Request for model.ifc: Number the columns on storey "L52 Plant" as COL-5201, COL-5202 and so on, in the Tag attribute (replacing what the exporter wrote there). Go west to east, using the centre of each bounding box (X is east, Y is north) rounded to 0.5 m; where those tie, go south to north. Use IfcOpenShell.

First a look at what the model holds.

```python
import ifcopenshell
import ifcopenshell.util.element
import ifcopenshell.util.placement

model = ifcopenshell.open("model.ifc")
print(model.schema)
storey = next(s for s in model.by_type("IfcBuildingStorey") if s.Name == "L52 Plant")
columns = [e for e in ifcopenshell.util.element.get_decomposition(storey) if e.is_a("IfcColumn")]
for e in sorted(columns, key=lambda e: e.id()):
    origin = ifcopenshell.util.placement.get_local_placement(e.ObjectPlacement)[:3, 3]
    print(e.id(), e.Tag, e.Name, origin.round(2) + 0.0, sep=" | ")
```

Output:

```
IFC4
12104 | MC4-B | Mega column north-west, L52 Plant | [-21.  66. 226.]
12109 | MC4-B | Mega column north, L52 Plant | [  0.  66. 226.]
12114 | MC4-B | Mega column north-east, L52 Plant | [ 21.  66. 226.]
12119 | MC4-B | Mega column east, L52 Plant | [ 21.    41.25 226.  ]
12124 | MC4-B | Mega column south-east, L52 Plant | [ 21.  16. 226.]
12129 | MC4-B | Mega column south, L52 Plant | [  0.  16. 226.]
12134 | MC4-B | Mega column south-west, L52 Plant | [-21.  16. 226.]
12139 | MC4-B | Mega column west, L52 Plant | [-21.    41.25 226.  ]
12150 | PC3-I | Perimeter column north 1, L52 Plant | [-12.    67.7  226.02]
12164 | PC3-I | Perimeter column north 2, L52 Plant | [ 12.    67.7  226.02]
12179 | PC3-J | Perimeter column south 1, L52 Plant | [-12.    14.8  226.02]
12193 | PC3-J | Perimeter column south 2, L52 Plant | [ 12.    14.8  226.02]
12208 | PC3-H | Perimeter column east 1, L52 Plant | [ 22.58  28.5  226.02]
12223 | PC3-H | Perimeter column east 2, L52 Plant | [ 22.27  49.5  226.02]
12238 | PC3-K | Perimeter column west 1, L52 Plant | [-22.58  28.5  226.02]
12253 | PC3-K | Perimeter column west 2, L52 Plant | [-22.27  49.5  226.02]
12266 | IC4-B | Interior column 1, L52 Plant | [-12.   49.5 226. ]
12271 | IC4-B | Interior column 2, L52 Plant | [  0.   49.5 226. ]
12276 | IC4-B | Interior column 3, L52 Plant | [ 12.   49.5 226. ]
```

```python
import ifcopenshell
import ifcopenshell.geom
import ifcopenshell.util.element
import ifcopenshell.util.shape

model = ifcopenshell.open("model.ifc")
settings = ifcopenshell.geom.settings()
settings.set("use-world-coords", True)


def centre(element):
    shape = ifcopenshell.geom.create_shape(settings, element)
    return ifcopenshell.util.shape.get_bbox_centroid(shape.geometry)


storey = next(s for s in model.by_type("IfcBuildingStorey") if s.Name == "L52 Plant")
columns = [e for e in ifcopenshell.util.element.get_decomposition(storey) if e.is_a("IfcColumn")]

# Insertion points can sit at a corner or the storey origin, so sort by the geometry (in metres).
centres = {e: centre(e) for e in columns}
columns.sort(key=lambda e: (round(centres[e][0] / 0.5), centres[e][1]))

for i, e in enumerate(columns, start=1):
    number = f"COL-52{i:02d}"
    e.Tag = number
    print(e.id(), number)

model.write("model_edited.ifc")
```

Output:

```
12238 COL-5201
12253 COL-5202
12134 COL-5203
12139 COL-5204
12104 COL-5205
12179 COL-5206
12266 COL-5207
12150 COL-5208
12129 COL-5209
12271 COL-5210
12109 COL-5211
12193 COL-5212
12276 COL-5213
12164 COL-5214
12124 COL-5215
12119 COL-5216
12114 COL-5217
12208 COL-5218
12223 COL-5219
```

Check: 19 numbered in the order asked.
